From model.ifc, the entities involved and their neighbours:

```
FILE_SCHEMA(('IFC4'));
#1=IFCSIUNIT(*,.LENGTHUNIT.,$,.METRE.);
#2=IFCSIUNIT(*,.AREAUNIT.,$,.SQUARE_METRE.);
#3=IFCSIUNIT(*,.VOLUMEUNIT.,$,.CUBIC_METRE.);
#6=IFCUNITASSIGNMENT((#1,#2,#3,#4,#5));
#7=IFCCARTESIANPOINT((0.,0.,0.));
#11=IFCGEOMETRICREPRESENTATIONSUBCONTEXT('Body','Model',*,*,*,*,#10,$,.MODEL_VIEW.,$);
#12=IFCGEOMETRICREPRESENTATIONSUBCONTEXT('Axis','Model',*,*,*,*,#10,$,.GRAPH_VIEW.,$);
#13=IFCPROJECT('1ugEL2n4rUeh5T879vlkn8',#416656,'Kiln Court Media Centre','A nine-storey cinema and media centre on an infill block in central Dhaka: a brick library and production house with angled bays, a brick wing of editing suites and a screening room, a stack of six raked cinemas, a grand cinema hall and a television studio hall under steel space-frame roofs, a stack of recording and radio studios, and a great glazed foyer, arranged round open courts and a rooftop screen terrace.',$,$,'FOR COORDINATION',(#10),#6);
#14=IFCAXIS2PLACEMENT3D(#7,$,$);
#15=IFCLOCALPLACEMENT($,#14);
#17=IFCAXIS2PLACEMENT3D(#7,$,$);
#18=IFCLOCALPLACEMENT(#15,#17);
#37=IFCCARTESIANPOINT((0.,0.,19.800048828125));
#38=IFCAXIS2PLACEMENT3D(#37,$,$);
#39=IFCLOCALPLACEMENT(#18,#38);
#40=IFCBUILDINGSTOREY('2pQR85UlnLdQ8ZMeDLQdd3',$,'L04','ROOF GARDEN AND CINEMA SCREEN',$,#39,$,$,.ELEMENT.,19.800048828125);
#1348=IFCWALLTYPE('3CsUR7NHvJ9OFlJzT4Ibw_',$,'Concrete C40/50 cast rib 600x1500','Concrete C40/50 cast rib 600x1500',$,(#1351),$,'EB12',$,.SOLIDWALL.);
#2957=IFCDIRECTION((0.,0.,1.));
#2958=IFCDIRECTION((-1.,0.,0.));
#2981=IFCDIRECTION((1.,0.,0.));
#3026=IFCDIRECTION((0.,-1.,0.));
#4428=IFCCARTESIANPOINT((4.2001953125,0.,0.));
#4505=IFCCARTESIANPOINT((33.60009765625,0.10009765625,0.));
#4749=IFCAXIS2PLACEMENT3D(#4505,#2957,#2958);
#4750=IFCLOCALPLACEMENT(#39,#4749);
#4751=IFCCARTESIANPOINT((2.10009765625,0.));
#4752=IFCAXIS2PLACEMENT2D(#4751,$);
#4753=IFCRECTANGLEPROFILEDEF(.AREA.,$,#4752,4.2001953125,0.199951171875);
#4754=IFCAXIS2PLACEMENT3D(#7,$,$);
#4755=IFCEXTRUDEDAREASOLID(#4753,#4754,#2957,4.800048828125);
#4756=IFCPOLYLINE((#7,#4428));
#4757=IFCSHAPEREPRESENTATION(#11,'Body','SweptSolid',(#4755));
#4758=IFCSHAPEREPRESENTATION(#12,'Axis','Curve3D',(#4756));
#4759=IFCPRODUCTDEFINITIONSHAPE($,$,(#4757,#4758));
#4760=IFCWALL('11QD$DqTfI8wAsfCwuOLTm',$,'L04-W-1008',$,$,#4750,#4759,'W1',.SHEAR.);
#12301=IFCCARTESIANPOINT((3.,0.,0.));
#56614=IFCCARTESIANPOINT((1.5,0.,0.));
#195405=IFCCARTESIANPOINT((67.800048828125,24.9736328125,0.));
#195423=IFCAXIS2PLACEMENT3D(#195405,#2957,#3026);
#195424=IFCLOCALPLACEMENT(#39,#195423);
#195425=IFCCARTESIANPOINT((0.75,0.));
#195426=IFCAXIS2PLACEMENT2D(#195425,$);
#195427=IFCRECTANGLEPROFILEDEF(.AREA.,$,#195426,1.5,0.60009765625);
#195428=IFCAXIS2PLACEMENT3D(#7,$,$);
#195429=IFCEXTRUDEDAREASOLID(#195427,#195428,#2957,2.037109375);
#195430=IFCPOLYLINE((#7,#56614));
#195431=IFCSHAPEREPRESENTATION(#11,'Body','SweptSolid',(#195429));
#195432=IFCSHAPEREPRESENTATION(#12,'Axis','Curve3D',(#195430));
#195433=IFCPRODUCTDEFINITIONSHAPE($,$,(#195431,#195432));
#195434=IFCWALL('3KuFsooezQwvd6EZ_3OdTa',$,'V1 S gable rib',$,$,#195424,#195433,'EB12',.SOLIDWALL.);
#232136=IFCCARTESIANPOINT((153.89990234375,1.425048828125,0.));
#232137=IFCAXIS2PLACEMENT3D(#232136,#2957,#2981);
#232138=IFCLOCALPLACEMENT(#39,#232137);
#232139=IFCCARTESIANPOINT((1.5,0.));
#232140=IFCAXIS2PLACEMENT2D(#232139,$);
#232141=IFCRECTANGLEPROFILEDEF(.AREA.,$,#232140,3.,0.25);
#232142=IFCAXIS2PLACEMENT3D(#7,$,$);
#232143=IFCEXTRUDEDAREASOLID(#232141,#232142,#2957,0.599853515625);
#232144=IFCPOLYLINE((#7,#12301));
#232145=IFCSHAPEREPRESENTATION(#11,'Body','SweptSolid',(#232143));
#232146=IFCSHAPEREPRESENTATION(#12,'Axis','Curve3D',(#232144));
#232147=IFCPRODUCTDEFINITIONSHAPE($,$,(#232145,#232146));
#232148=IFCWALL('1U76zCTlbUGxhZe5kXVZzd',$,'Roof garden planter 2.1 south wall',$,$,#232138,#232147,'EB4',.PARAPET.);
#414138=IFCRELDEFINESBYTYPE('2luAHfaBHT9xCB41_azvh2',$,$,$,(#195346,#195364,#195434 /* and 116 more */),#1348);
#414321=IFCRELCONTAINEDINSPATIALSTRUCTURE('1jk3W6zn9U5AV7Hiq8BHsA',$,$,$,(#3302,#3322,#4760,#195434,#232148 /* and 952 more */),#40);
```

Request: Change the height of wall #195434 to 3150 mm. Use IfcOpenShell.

```python
import ifcopenshell
import ifcopenshell.geom
import ifcopenshell.util.representation
import ifcopenshell.util.shape
import ifcopenshell.util.unit

model = ifcopenshell.open("model.ifc")
unit_scale = ifcopenshell.util.unit.calculate_unit_scale(model)
settings = ifcopenshell.geom.settings()


def volume(element):
    """Net volume in cubic metres, openings subtracted."""
    shape = ifcopenshell.geom.create_shape(settings, element)
    return ifcopenshell.util.shape.get_volume(shape.geometry)


wall = model.by_guid("3KuFsooezQwvd6EZ_3OdTa")
before = volume(wall)

body = ifcopenshell.util.representation.get_representation(wall, "Model", "Body")
solid = body.Items[0]
old_height = solid.Depth
solid.Depth = 3.15 / unit_scale
after = volume(wall)

print(f"height {old_height:g} -> {solid.Depth:g}, volume {before:.3f} -> {after:.3f} m3")

model.write("model_updated.ifc")
```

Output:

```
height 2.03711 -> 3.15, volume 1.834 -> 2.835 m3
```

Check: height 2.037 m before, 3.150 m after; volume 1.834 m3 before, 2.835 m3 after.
